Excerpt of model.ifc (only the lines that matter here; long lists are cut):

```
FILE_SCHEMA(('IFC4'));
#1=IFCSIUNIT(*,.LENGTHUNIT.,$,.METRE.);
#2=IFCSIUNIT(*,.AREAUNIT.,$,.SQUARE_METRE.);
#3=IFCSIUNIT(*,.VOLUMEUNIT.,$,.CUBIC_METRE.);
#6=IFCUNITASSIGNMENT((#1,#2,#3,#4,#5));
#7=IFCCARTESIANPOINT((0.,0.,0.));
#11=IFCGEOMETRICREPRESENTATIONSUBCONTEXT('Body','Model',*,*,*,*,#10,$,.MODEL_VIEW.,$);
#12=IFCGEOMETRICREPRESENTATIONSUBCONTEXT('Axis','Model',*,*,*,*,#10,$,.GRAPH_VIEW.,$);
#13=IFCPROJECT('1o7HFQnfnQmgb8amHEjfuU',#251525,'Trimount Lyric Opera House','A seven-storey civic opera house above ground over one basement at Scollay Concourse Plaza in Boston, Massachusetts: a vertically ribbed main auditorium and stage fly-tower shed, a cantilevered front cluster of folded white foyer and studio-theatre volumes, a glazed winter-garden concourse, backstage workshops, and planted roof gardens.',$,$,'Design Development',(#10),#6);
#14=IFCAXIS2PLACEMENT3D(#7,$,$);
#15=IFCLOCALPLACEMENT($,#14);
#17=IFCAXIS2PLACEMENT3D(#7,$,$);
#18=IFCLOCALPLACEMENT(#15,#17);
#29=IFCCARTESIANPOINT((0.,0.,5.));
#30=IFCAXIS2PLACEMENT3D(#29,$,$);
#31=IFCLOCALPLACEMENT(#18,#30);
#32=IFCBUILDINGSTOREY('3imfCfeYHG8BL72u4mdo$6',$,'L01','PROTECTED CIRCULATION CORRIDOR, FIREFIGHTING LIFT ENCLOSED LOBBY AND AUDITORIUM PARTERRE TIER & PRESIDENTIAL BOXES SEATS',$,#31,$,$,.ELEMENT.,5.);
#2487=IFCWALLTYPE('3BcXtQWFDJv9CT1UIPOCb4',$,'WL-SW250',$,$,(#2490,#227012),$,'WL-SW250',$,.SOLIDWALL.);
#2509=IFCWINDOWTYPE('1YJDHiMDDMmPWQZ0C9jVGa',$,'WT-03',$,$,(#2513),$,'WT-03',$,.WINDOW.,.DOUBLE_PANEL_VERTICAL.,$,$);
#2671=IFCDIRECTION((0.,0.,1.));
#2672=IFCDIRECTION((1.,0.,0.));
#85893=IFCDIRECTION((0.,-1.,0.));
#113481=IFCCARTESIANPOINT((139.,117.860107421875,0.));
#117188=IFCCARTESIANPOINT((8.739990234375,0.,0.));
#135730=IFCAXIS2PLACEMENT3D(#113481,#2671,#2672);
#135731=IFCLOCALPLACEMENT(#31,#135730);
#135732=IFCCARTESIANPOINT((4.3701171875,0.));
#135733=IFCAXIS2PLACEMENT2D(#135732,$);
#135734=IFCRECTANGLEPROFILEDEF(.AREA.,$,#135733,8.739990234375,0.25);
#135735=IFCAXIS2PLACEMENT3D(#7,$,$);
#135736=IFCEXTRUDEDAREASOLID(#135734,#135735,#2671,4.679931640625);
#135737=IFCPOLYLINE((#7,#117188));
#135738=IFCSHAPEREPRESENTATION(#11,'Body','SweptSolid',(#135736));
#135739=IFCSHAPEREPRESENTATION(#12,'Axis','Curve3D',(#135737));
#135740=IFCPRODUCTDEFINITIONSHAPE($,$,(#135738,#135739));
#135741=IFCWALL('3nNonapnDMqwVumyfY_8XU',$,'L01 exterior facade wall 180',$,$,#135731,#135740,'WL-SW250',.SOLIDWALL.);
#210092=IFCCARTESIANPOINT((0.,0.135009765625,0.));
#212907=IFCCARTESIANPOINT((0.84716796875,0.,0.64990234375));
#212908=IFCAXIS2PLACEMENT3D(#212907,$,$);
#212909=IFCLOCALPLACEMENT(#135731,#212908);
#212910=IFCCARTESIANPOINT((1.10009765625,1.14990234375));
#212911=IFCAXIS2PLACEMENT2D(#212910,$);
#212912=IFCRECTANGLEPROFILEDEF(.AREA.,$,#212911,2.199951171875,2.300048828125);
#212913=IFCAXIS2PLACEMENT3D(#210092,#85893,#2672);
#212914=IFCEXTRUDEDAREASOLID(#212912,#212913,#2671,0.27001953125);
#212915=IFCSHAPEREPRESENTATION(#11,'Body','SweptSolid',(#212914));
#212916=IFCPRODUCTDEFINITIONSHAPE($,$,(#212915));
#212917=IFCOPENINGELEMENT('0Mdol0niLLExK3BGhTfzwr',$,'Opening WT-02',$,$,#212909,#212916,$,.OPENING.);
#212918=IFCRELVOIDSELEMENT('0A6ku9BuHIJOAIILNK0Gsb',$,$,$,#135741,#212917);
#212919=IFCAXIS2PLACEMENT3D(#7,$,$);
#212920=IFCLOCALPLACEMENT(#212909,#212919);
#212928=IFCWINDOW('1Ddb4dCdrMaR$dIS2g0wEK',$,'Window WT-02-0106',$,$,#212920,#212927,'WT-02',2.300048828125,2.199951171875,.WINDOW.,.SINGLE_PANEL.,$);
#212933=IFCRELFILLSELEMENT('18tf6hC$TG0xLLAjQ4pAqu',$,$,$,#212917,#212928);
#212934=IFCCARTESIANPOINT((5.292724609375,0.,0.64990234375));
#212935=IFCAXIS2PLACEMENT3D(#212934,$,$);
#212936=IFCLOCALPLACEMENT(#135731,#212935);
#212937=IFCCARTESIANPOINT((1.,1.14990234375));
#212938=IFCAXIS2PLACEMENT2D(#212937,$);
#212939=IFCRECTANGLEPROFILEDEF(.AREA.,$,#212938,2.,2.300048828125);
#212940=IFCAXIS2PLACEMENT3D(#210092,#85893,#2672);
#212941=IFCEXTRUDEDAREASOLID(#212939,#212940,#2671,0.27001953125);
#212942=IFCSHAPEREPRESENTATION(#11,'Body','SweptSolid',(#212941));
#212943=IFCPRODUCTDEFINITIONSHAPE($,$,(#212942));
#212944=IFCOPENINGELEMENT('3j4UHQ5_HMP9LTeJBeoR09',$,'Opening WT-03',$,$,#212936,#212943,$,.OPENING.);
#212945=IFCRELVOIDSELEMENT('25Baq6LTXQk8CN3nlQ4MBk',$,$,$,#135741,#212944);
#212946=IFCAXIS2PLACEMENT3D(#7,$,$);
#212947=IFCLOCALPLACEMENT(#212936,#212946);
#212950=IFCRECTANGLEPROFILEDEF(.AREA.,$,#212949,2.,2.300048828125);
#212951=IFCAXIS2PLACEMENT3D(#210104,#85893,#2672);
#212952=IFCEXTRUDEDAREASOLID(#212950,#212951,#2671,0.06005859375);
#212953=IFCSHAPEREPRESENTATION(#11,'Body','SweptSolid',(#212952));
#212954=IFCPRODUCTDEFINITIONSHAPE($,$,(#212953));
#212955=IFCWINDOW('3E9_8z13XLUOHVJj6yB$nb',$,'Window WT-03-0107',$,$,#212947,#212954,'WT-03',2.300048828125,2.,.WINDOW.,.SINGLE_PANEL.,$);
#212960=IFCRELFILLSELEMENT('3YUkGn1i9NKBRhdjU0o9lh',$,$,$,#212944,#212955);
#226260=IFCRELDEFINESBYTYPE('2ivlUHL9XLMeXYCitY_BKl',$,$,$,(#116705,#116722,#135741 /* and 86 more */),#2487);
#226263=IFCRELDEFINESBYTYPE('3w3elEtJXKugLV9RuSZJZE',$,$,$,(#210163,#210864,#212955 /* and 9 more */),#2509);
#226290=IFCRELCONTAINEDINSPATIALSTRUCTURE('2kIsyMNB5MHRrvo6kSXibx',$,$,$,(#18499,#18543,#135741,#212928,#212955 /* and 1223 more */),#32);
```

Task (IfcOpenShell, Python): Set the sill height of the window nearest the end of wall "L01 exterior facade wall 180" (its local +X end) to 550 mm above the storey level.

```python
import numpy as np
import ifcopenshell
import ifcopenshell.api.geometry
import ifcopenshell.geom
import ifcopenshell.util.element
import ifcopenshell.util.placement
import ifcopenshell.util.shape
import ifcopenshell.util.unit

model = ifcopenshell.open("model.ifc")
unit_scale = ifcopenshell.util.unit.calculate_unit_scale(model)

window = model.by_id(212955)
opening = window.FillsVoids[0].RelatingOpeningElement
storey = ifcopenshell.util.element.get_container(window, ifc_class="IfcBuildingStorey")
level = ifcopenshell.util.placement.get_local_placement(storey.ObjectPlacement)[2, 3]

# The opening's origin need not be at the sill, so measure its lowest point.
shape = ifcopenshell.geom.create_shape(ifcopenshell.geom.settings(), opening)
bottom = ifcopenshell.util.shape.get_shape_bottom_elevation(shape, shape.geometry) / unit_scale
dz = level + 0.55 / unit_scale - bottom

shift = np.array([0.0, 0.0, dz])
# The window is placed relative to its opening, so it follows when the opening moves.
matrix = ifcopenshell.util.placement.get_local_placement(opening.ObjectPlacement)
matrix[:3, 3] += shift
ifcopenshell.api.geometry.edit_object_placement(
    model, product=opening, matrix=matrix, is_si=False, should_transform_children=True
)

print(f"moved by {dz * unit_scale:+.3f} m")

model.write("model-out.ifc")
```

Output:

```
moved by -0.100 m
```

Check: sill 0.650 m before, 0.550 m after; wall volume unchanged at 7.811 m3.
